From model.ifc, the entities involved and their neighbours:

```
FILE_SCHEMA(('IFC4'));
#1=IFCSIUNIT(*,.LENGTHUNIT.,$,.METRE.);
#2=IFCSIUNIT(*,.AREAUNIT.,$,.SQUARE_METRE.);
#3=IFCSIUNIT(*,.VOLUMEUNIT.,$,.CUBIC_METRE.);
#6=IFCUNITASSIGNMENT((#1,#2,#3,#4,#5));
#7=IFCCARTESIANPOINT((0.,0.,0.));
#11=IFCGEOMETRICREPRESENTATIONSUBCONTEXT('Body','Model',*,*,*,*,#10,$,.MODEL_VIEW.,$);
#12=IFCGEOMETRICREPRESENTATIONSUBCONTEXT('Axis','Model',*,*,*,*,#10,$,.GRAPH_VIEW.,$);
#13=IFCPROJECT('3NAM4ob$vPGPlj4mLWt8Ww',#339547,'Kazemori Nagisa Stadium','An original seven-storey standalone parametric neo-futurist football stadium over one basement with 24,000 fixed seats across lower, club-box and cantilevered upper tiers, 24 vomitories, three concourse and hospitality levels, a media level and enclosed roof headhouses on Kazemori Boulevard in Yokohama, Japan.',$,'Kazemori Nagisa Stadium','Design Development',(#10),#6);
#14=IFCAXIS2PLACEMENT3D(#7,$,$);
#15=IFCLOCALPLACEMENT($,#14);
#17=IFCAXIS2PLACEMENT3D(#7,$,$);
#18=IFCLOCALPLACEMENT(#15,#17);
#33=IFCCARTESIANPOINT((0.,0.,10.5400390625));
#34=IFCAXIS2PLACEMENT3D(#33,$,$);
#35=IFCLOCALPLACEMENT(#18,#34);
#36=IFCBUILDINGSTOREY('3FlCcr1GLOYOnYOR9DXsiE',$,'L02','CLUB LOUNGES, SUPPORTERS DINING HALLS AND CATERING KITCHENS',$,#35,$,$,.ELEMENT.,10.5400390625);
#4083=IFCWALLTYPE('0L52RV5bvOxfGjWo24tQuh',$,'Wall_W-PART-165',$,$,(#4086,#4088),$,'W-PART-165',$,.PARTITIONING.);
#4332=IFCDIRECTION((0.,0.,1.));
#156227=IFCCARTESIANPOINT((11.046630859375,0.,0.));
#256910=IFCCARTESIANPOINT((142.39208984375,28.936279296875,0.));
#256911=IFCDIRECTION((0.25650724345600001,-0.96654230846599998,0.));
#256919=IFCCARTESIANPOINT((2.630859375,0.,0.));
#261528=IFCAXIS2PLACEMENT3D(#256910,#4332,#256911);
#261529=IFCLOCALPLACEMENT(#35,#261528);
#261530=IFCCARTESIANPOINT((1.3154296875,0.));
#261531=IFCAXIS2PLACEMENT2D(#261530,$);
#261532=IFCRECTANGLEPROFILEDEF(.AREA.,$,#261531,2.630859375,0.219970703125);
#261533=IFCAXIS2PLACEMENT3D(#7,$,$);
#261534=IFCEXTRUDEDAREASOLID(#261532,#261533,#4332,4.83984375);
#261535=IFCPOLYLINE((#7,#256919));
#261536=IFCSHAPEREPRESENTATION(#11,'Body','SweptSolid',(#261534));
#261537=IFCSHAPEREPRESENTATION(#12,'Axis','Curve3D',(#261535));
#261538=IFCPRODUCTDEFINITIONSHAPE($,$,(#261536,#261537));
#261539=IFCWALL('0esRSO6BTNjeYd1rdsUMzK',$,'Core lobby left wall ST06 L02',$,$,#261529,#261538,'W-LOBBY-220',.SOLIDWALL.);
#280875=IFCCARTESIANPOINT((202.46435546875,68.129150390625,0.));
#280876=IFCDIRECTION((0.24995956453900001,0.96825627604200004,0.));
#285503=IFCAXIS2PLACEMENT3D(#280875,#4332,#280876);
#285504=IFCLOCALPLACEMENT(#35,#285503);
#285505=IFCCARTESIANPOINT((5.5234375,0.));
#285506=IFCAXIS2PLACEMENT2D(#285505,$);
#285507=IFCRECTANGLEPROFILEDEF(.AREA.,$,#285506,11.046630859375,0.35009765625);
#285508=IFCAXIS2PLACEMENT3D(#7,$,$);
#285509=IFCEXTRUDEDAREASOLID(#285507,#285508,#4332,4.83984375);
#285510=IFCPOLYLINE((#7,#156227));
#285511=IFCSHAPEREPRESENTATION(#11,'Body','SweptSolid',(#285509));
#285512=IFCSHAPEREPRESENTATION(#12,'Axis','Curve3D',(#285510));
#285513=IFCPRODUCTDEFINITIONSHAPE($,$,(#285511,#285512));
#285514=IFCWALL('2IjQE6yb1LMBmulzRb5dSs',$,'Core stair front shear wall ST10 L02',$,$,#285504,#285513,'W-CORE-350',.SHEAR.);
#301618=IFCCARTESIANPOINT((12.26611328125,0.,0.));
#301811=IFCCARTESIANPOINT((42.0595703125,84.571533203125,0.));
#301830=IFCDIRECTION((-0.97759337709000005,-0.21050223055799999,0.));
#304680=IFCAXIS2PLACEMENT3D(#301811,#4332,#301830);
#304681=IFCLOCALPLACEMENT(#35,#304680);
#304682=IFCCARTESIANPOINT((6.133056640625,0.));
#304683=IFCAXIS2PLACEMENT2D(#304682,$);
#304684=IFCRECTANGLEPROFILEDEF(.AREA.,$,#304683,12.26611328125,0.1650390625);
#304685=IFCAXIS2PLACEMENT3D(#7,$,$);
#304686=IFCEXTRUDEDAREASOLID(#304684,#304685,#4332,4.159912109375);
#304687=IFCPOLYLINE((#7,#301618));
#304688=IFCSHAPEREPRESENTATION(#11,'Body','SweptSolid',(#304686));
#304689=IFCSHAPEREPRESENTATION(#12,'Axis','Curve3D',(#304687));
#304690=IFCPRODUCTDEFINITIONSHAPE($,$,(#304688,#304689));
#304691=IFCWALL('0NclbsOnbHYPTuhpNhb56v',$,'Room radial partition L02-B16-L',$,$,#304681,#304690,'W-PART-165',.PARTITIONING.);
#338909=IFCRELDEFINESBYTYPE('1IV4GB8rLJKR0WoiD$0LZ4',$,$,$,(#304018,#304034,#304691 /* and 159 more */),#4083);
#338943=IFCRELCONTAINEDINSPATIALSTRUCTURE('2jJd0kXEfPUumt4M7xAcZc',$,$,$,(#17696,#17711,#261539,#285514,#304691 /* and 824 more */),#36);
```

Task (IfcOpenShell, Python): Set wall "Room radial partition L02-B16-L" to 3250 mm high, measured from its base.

```python
import ifcopenshell
import ifcopenshell.geom
import ifcopenshell.util.representation
import ifcopenshell.util.shape
import ifcopenshell.util.unit

model = ifcopenshell.open("model.ifc")
unit_scale = ifcopenshell.util.unit.calculate_unit_scale(model)
settings = ifcopenshell.geom.settings()


def volume(element):
    """Net volume in cubic metres, openings subtracted."""
    shape = ifcopenshell.geom.create_shape(settings, element)
    return ifcopenshell.util.shape.get_volume(shape.geometry)


wall = model.by_guid("0NclbsOnbHYPTuhpNhb56v")
before = volume(wall)

body = ifcopenshell.util.representation.get_representation(wall, "Model", "Body")
solid = body.Items[0]
old_height = solid.Depth
solid.Depth = 3.25 / unit_scale
after = volume(wall)

print(f"height {old_height:g} -> {solid.Depth:g}, volume {before:.3f} -> {after:.3f} m3")

model.write("model-out.ifc")
```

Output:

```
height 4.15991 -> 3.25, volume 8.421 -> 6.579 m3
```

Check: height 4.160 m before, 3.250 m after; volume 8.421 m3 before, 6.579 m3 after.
